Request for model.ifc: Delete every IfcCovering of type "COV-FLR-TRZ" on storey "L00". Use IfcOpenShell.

First a look at what the model holds.

```python
import ifcopenshell
import ifcopenshell.util.element

model = ifcopenshell.open("model.ifc")
print(model.schema)
storey = next(s for s in model.by_type("IfcBuildingStorey") if s.Name == "L00")
coverings = [e for e in ifcopenshell.util.element.get_decomposition(storey) if e.is_a("IfcCovering")]
seen = {}
for e in coverings:
    element_type = ifcopenshell.util.element.get_type(e)
    name = element_type.Name if element_type not in (None, e) else None
    seen[name] = seen.get(name, 0) + 1
for name, count in sorted(seen.items(), key=str):
    print(count, "x", name)
```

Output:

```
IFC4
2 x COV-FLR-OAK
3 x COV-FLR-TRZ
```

```python
import ifcopenshell
import ifcopenshell.api.root
import ifcopenshell.util.element

model = ifcopenshell.open("model.ifc")

storey = next(s for s in model.by_type("IfcBuildingStorey") if s.Name == "L00")
coverings = [e for e in ifcopenshell.util.element.get_decomposition(storey) if e.is_a("IfcCovering")]
targets = [e for e in coverings if (t := ifcopenshell.util.element.get_type(e)) not in (None, e) and t.Name == "COV-FLR-TRZ"]

for e in targets:
    ifcopenshell.api.root.remove_product(model, product=e)
print(len(targets), "removed")

model.write("model-out.ifc")
```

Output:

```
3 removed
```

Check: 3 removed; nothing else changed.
